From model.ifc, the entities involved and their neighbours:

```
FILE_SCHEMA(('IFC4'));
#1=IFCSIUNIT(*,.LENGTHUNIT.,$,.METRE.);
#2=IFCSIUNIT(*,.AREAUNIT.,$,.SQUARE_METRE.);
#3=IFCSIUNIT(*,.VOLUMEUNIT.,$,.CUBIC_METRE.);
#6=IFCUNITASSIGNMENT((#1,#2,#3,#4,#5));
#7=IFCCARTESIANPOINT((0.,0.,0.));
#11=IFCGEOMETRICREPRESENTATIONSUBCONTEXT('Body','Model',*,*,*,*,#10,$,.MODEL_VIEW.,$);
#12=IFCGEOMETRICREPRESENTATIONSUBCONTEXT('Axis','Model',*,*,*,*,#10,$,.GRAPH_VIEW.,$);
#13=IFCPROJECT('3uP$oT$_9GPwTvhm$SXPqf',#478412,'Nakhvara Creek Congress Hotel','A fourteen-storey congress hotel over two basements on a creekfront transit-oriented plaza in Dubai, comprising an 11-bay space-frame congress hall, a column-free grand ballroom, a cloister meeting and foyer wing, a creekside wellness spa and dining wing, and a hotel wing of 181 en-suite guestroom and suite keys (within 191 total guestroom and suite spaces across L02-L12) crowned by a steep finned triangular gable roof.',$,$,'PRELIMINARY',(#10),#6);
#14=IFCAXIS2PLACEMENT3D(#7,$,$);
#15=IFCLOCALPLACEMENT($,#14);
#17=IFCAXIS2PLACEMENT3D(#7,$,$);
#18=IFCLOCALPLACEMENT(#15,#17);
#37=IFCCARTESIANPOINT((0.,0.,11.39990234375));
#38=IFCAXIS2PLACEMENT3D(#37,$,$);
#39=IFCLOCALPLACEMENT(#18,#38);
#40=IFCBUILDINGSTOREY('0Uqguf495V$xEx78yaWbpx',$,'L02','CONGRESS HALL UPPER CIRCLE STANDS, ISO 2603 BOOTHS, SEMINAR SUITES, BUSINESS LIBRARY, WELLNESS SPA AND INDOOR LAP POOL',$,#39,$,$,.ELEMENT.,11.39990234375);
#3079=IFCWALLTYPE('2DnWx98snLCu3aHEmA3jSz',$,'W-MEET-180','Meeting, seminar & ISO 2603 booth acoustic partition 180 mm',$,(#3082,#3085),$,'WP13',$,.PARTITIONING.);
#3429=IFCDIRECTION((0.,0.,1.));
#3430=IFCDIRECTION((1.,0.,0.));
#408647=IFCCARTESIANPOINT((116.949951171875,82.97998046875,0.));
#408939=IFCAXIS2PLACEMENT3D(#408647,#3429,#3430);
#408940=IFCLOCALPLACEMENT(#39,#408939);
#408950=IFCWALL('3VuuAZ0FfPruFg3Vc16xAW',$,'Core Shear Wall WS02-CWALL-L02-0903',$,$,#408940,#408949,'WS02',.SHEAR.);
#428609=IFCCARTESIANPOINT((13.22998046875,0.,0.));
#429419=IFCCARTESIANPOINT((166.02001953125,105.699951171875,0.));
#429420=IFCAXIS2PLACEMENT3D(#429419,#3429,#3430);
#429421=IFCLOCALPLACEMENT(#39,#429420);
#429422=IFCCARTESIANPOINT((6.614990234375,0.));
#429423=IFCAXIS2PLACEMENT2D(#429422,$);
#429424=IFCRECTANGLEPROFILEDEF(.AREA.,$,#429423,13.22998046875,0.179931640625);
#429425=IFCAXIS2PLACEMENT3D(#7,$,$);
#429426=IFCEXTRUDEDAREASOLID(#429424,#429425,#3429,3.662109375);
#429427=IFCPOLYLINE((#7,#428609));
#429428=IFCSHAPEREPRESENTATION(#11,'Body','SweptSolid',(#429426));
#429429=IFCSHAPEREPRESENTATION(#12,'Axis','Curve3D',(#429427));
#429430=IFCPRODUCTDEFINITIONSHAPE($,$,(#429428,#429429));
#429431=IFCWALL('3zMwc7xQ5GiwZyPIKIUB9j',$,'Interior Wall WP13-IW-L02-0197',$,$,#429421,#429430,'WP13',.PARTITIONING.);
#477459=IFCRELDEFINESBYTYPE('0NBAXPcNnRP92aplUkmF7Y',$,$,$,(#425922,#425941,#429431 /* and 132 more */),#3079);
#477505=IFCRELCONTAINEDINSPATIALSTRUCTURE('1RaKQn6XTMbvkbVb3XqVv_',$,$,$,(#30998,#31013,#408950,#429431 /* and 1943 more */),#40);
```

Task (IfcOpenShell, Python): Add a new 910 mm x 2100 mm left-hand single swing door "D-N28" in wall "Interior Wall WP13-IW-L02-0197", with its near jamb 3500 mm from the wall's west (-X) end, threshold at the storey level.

```python
import numpy as np
import ifcopenshell
import ifcopenshell.api.feature
import ifcopenshell.api.geometry
import ifcopenshell.api.root
import ifcopenshell.api.spatial
import ifcopenshell.geom
import ifcopenshell.util.element
import ifcopenshell.util.placement
import ifcopenshell.util.representation
import ifcopenshell.util.shape
import ifcopenshell.util.unit

model = ifcopenshell.open("model.ifc")
unit_scale = ifcopenshell.util.unit.calculate_unit_scale(model)
settings = ifcopenshell.geom.settings()


def volume(element):
    """Net volume in cubic metres, openings subtracted."""
    shape = ifcopenshell.geom.create_shape(settings, element)
    return ifcopenshell.util.shape.get_volume(shape.geometry)


wall = model.by_guid("3zMwc7xQ5GiwZyPIKIUB9j")
storey = ifcopenshell.util.element.get_container(wall, ifc_class="IfcBuildingStorey")
context = ifcopenshell.util.representation.get_context(model, "Model", "Body", "MODEL_VIEW")
before = volume(wall)

width, height, from_end, sill = 0.91, 2.1, 3.5, 0.0  # metres

# The wall runs along its own X axis, and the end named is its -X end.
wall_shape = ifcopenshell.geom.create_shape(settings, wall)
x, y, z = ifcopenshell.util.shape.get_vertices(wall_shape.geometry).T
start = x.min() + from_end
face, thickness = float(y.min()), float(y.max() - y.min())
wall_matrix = ifcopenshell.util.placement.get_local_placement(wall.ObjectPlacement)
level = ifcopenshell.util.placement.get_local_placement(storey.ObjectPlacement)[2, 3]


def in_wall(x, y):
    """Placement at x, y metres in the wall's axes, at sill height."""
    matrix = wall_matrix.copy()
    matrix[:, 3] = wall_matrix @ np.array([x / unit_scale, y / unit_scale, 0.0, 1.0])
    matrix[2, 3] = level + sill / unit_scale
    return matrix


# Opening: a box that overshoots both wall faces by 50 mm.
opening = ifcopenshell.api.root.create_entity(model, ifc_class="IfcOpeningElement", predefined_type="OPENING")
box = ifcopenshell.api.geometry.add_wall_representation(
    model, context=context, length=width, height=height, thickness=thickness + 0.1
)
ifcopenshell.api.geometry.assign_representation(model, product=opening, representation=box)
ifcopenshell.api.geometry.edit_object_placement(model, product=opening, matrix=in_wall(start, face - 0.05), is_si=False)
ifcopenshell.api.feature.add_feature(model, feature=opening, element=wall)

door = ifcopenshell.api.root.create_entity(model, ifc_class="IfcDoor", name="D-N28", predefined_type="DOOR")
door.OverallWidth, door.OverallHeight = width / unit_scale, height / unit_scale
door.OperationType = "SINGLE_SWING_LEFT"
body = ifcopenshell.api.geometry.add_door_representation(
    model,
    context=context,
    overall_width=door.OverallWidth,
    overall_height=door.OverallHeight,
    operation_type="SINGLE_SWING_LEFT",
    lining_properties={"LiningDepth": thickness / unit_scale, "ThresholdDepth": thickness / unit_scale},
)
ifcopenshell.api.geometry.assign_representation(model, product=door, representation=body)
ifcopenshell.api.spatial.assign_container(model, products=[door], relating_structure=storey)
ifcopenshell.api.feature.add_filling(model, opening=opening, element=door)

# The lining spans the wall, so the door starts at the wall face.
ifcopenshell.api.geometry.edit_object_placement(model, product=door, matrix=in_wall(start, face), is_si=False)

after = volume(wall)

print(f"wall volume {before:.3f} -> {after:.3f} m3")

model.write("model_edited.ifc")
```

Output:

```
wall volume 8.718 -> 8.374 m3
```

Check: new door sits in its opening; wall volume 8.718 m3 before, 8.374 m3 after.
